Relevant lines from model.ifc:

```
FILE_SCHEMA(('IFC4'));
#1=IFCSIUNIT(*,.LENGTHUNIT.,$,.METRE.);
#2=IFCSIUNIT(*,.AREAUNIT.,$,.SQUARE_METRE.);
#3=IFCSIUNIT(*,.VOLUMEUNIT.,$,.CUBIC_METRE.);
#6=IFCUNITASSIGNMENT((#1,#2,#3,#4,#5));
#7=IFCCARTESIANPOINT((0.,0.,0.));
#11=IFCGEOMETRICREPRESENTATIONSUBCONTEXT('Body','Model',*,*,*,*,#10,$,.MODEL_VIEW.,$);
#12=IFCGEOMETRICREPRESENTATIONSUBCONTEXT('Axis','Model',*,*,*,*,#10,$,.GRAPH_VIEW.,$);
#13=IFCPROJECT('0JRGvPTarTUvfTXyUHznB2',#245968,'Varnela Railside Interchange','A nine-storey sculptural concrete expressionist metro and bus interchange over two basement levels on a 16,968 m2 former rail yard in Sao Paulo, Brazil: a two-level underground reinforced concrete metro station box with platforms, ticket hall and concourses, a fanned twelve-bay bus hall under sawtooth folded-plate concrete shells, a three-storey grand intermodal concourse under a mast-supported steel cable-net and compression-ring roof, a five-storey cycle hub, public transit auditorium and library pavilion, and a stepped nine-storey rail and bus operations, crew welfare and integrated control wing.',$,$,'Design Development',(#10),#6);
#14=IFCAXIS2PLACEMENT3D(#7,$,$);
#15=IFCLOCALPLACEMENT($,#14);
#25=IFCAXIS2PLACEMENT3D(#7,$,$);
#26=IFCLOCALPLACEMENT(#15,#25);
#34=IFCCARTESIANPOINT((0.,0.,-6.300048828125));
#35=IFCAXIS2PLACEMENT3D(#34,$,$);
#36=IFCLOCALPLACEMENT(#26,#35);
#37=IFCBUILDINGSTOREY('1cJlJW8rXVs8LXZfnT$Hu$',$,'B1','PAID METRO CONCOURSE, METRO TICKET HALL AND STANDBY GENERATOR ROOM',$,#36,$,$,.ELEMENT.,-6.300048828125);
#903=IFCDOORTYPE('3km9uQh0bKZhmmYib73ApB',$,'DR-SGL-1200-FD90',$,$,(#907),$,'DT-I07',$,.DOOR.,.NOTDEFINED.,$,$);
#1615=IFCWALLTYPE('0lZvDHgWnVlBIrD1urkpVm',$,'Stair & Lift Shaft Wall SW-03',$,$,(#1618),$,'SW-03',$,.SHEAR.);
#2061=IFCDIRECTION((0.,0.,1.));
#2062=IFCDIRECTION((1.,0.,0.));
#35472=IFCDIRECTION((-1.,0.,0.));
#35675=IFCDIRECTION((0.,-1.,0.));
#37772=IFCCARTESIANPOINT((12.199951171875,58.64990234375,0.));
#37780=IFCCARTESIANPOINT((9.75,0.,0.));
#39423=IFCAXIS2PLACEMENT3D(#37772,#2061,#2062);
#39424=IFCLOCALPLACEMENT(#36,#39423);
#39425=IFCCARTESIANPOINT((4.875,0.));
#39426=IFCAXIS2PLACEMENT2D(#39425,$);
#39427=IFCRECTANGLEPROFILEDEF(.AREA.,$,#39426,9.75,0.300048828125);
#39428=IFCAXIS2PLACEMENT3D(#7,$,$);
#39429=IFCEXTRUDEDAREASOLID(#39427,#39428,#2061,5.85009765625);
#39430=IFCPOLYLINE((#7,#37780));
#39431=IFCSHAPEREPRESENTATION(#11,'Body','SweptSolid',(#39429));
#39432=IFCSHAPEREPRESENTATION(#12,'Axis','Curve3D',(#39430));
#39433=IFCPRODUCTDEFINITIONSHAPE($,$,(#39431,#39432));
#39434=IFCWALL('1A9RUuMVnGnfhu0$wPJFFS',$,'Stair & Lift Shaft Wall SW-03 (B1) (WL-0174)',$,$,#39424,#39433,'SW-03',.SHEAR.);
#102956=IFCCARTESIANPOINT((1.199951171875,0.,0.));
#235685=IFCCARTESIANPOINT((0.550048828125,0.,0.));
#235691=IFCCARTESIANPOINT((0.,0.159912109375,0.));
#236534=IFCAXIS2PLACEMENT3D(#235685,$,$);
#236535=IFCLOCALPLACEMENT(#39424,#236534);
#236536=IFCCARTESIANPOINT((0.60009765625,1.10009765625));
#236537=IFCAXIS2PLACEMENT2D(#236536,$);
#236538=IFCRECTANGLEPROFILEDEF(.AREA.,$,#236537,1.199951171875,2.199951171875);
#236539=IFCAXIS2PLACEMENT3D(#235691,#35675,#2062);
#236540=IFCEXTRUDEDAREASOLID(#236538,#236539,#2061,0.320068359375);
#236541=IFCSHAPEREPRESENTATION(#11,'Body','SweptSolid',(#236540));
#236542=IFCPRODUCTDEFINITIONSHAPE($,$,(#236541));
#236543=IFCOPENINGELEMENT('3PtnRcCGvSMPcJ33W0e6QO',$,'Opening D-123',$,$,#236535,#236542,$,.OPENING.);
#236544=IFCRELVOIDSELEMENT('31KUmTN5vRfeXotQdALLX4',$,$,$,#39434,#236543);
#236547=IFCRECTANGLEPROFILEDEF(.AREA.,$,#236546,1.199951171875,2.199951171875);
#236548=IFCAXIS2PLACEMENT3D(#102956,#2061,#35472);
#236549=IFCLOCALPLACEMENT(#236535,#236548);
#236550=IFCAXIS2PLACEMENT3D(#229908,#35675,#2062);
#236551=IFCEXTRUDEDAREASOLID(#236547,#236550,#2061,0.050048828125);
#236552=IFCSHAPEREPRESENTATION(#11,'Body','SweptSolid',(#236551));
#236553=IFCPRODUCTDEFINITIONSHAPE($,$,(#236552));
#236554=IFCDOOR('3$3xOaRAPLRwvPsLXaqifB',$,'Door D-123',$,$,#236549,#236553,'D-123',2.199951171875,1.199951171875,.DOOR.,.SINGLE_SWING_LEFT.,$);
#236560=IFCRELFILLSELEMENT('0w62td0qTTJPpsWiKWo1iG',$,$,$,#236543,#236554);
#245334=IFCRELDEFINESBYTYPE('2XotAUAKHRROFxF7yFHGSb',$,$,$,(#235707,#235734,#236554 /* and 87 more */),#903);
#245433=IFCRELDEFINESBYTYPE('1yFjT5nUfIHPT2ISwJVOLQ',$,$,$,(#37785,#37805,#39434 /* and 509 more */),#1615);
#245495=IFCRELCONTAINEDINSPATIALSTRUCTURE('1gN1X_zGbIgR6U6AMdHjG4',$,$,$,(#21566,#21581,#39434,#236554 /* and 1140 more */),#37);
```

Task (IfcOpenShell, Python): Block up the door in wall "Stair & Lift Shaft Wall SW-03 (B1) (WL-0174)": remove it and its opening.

```python
import ifcopenshell
import ifcopenshell.api.feature
import ifcopenshell.api.root
import ifcopenshell.geom
import ifcopenshell.util.shape

model = ifcopenshell.open("model.ifc")
settings = ifcopenshell.geom.settings()


def volume(element):
    """Net volume in cubic metres, openings subtracted."""
    shape = ifcopenshell.geom.create_shape(settings, element)
    return ifcopenshell.util.shape.get_volume(shape.geometry)


door = model.by_guid("3$3xOaRAPLRwvPsLXaqifB")
opening = door.FillsVoids[0].RelatingOpeningElement
wall = opening.VoidsElements[0].RelatingBuildingElement
before = volume(wall)

ifcopenshell.api.root.remove_product(model, product=door)
ifcopenshell.api.feature.remove_feature(model, feature=opening)

after = volume(wall)

print(f"wall volume {before:.3f} -> {after:.3f} m3")

model.write("model_edited.ifc")
```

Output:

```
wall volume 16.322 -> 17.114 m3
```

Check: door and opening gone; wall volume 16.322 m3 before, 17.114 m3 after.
